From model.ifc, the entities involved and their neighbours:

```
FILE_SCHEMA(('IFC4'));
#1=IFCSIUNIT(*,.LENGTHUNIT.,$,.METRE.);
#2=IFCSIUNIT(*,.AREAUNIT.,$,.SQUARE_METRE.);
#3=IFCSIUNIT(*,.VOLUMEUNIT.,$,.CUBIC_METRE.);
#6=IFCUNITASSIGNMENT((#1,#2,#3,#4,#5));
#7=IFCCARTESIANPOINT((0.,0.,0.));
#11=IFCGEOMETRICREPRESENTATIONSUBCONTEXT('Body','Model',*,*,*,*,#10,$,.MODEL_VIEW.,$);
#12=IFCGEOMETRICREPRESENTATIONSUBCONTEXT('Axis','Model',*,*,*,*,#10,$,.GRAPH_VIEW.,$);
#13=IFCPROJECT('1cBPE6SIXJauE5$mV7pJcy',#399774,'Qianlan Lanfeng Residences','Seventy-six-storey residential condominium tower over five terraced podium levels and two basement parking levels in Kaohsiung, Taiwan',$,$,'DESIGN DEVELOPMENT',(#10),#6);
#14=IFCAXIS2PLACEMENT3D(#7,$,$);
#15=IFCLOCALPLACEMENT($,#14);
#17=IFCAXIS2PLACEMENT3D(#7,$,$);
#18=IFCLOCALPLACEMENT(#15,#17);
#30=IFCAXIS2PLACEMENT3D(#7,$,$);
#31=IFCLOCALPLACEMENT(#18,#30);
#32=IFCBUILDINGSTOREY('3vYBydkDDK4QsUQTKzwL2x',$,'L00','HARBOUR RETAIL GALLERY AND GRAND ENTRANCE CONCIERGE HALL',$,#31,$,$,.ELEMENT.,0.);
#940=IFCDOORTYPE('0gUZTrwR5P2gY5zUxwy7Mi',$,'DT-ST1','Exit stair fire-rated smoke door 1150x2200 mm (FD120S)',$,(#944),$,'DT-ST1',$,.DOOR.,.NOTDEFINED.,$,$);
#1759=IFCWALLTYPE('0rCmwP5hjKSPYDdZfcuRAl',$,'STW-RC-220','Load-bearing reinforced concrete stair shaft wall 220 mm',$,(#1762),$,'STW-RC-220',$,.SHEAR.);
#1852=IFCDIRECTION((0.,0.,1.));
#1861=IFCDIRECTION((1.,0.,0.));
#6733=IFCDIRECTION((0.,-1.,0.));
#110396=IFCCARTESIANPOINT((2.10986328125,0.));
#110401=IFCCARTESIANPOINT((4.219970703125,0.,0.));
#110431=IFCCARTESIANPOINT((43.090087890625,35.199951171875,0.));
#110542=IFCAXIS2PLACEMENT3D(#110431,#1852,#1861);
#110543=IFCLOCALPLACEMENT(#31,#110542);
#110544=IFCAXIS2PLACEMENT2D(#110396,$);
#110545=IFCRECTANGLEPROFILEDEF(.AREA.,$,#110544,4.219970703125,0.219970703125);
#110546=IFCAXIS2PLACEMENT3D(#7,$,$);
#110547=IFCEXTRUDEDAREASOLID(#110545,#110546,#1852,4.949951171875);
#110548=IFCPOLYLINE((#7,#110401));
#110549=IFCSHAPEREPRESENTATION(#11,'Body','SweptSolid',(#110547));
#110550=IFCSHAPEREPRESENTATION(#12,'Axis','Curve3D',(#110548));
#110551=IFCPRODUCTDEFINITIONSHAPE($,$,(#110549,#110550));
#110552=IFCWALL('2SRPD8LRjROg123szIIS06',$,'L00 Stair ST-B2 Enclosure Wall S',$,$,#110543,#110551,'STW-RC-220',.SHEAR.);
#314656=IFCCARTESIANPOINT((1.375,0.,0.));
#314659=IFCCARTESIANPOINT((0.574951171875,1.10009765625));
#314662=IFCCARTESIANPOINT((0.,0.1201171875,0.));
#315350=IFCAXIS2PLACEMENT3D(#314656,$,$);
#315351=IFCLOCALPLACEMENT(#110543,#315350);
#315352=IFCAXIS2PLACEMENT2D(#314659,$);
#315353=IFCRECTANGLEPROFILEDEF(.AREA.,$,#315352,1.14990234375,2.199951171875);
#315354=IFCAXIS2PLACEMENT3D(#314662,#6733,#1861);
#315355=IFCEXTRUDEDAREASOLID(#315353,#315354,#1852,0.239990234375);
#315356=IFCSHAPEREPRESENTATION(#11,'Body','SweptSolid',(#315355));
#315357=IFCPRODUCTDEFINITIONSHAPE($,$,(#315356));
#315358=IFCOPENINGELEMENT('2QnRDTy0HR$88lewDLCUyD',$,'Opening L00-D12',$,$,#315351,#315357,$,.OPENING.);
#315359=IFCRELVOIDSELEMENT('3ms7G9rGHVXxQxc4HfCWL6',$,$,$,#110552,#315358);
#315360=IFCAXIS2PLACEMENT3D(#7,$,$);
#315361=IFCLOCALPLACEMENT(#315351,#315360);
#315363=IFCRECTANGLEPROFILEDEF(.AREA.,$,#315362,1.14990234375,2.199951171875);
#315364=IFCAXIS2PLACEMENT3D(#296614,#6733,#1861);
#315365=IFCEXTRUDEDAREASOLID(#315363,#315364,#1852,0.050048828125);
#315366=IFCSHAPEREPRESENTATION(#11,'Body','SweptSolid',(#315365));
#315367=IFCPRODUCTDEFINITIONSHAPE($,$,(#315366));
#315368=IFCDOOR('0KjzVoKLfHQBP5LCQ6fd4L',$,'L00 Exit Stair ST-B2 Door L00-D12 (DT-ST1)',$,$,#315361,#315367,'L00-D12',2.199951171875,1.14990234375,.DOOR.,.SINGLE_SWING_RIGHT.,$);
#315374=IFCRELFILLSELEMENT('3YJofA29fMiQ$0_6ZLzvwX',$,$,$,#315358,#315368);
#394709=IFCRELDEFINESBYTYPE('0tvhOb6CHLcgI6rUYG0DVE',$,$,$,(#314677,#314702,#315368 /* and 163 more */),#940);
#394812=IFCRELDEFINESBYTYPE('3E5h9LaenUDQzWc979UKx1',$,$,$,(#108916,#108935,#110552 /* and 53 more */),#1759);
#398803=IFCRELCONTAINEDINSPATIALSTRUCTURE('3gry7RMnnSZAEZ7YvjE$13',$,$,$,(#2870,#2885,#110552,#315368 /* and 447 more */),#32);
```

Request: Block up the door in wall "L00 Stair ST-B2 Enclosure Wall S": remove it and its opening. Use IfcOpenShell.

```python
import ifcopenshell
import ifcopenshell.api.feature
import ifcopenshell.api.root
import ifcopenshell.geom
import ifcopenshell.util.shape

model = ifcopenshell.open("model.ifc")
settings = ifcopenshell.geom.settings()


def volume(element):
    """Net volume in cubic metres, openings subtracted."""
    shape = ifcopenshell.geom.create_shape(settings, element)
    return ifcopenshell.util.shape.get_volume(shape.geometry)


door = model.by_guid("0KjzVoKLfHQBP5LCQ6fd4L")
opening = door.FillsVoids[0].RelatingOpeningElement
wall = opening.VoidsElements[0].RelatingBuildingElement
before = volume(wall)

ifcopenshell.api.root.remove_product(model, product=door)
ifcopenshell.api.feature.remove_feature(model, feature=opening)

after = volume(wall)

print(f"wall volume {before:.3f} -> {after:.3f} m3")

model.write("model_edited.ifc")
```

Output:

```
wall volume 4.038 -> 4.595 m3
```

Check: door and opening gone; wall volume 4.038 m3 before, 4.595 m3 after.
